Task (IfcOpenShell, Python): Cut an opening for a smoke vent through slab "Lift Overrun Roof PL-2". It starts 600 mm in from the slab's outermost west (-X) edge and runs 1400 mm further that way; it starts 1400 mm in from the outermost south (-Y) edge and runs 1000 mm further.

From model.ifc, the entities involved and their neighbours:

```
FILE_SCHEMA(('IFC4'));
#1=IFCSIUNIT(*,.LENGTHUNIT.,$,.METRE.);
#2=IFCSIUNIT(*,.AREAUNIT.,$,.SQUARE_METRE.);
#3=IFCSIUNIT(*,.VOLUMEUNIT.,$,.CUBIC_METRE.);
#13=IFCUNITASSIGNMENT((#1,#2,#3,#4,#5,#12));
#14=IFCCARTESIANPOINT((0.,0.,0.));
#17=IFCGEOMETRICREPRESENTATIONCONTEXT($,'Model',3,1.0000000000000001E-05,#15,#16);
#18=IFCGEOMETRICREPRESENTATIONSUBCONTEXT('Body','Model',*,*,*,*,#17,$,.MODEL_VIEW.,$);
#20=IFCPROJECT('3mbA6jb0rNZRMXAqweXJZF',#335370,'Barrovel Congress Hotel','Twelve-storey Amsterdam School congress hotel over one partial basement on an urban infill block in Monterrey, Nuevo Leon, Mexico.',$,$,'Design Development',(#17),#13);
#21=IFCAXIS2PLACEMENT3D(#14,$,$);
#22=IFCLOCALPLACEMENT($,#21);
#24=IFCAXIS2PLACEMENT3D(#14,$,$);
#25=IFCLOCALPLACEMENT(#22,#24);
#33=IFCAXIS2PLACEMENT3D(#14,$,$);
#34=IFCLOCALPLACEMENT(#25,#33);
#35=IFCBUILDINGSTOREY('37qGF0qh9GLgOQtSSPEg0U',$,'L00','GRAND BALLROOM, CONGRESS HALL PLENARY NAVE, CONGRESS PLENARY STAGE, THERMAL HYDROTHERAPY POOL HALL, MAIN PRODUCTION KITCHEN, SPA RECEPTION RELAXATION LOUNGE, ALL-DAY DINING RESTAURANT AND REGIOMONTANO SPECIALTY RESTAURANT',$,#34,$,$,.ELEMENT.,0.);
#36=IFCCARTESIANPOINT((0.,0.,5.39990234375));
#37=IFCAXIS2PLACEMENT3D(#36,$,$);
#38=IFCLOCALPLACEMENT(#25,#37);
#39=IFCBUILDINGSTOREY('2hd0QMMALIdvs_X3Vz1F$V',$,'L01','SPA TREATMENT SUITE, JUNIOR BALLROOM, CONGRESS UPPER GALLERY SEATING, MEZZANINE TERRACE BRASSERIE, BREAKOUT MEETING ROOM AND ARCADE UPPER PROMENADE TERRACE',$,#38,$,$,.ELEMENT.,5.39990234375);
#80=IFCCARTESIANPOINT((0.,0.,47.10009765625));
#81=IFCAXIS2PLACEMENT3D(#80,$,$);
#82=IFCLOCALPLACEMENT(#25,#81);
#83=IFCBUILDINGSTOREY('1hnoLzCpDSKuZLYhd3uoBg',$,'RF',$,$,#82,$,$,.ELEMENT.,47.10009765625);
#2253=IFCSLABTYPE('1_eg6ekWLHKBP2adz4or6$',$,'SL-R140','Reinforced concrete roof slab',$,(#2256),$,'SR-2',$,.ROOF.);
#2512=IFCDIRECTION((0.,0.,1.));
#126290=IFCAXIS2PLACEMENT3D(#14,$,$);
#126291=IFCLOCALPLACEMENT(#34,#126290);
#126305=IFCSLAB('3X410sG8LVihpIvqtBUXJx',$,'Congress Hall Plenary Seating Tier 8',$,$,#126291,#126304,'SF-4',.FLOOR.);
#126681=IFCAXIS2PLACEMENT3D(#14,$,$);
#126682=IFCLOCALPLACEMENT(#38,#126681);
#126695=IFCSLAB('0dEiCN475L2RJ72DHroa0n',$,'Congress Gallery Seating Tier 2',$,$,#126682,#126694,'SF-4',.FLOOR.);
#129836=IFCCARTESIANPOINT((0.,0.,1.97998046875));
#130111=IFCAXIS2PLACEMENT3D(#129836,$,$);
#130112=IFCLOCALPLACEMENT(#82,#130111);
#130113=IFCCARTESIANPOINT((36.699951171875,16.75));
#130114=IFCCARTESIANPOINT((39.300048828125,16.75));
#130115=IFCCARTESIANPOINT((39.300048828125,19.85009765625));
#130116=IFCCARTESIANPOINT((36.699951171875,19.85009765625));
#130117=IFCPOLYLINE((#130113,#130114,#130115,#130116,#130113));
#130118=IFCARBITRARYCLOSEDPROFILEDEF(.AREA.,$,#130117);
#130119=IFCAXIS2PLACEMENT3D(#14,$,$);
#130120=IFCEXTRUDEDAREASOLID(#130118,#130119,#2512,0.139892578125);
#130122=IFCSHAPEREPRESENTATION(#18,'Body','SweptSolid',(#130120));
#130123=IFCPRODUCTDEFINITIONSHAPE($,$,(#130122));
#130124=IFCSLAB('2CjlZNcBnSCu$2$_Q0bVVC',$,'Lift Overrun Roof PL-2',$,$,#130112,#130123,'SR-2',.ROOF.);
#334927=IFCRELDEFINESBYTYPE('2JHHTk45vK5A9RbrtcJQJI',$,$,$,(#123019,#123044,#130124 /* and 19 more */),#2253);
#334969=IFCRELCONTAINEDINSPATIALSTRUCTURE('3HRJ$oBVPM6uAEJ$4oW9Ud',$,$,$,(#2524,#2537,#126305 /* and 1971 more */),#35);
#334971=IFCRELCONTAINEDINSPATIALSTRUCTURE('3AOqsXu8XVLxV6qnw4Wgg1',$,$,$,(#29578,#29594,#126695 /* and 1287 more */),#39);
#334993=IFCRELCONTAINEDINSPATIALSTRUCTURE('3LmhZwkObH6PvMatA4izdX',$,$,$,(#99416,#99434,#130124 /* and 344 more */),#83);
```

```python
import numpy as np
import ifcopenshell
import ifcopenshell.api.feature
import ifcopenshell.api.geometry
import ifcopenshell.api.root
import ifcopenshell.geom
import ifcopenshell.util.placement
import ifcopenshell.util.representation
import ifcopenshell.util.shape
import ifcopenshell.util.unit

model = ifcopenshell.open("model.ifc")
unit_scale = ifcopenshell.util.unit.calculate_unit_scale(model)
settings = ifcopenshell.geom.settings()


def volume(element):
    """Net volume in cubic metres, openings subtracted."""
    shape = ifcopenshell.geom.create_shape(settings, element)
    return ifcopenshell.util.shape.get_volume(shape.geometry)


slab = model.by_guid("2CjlZNcBnSCu$2$_Q0bVVC")
before = volume(slab)

# Extent in the slab's own axes, in metres. The edges named are its -X and -Y sides.
slab_shape = ifcopenshell.geom.create_shape(settings, slab)
vertices = ifcopenshell.util.shape.get_vertices(slab_shape.geometry)
x_min, y_min, bottom = vertices.min(axis=0)
top = vertices[:, 2].max()

opening = ifcopenshell.api.root.create_entity(model, ifc_class="IfcOpeningElement", name="Smoke vent opening", predefined_type="OPENING")
context = ifcopenshell.util.representation.get_context(model, "Model", "Body", "MODEL_VIEW")
width, depth = 1.4, 1
outline = [(0.0, 0.0), (width, 0.0), (width, depth), (0.0, depth), (0.0, 0.0)]
# Overshoot both faces by 50 mm so the cut is clean.
shape = ifcopenshell.api.geometry.add_slab_representation(
    model, context=context, depth=top - bottom + 0.1, polyline=outline
)
ifcopenshell.api.geometry.assign_representation(model, product=opening, representation=shape)

matrix = ifcopenshell.util.placement.get_local_placement(slab.ObjectPlacement)
matrix[:, 3] = matrix @ np.append(np.array([x_min + 0.6, y_min + 1.4, bottom - 0.05]) / unit_scale, 1.0)
ifcopenshell.api.geometry.edit_object_placement(model, product=opening, matrix=matrix, is_si=False)
ifcopenshell.api.feature.add_feature(model, feature=opening, element=slab)

after = volume(slab)

print(f"slab volume {before:.3f} -> {after:.3f} m3")

model.write("model_edited.ifc")
```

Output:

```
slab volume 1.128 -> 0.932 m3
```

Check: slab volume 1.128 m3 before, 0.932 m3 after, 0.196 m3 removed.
